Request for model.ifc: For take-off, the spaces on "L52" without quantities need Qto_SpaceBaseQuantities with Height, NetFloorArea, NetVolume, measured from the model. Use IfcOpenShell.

First a look at what the model holds.

```python
import ifcopenshell
import ifcopenshell.util.element
import ifcopenshell.util.unit

model = ifcopenshell.open("model.ifc")
print(model.schema)
for unit_type in ("LENGTHUNIT", "AREAUNIT", "VOLUMEUNIT"):
    print(unit_type, ifcopenshell.util.unit.calculate_unit_scale(model, unit_type))
storey = next(s for s in model.by_type("IfcBuildingStorey") if s.Name == "L52")
spaces = [e for e in ifcopenshell.util.element.get_decomposition(storey) if e.is_a("IfcSpace")]
for e in sorted(spaces, key=lambda e: e.id()):
    print(e.id(), e.is_a(), e.Name, list(ifcopenshell.util.element.get_psets(e, qtos_only=True)), sep=" | ")
```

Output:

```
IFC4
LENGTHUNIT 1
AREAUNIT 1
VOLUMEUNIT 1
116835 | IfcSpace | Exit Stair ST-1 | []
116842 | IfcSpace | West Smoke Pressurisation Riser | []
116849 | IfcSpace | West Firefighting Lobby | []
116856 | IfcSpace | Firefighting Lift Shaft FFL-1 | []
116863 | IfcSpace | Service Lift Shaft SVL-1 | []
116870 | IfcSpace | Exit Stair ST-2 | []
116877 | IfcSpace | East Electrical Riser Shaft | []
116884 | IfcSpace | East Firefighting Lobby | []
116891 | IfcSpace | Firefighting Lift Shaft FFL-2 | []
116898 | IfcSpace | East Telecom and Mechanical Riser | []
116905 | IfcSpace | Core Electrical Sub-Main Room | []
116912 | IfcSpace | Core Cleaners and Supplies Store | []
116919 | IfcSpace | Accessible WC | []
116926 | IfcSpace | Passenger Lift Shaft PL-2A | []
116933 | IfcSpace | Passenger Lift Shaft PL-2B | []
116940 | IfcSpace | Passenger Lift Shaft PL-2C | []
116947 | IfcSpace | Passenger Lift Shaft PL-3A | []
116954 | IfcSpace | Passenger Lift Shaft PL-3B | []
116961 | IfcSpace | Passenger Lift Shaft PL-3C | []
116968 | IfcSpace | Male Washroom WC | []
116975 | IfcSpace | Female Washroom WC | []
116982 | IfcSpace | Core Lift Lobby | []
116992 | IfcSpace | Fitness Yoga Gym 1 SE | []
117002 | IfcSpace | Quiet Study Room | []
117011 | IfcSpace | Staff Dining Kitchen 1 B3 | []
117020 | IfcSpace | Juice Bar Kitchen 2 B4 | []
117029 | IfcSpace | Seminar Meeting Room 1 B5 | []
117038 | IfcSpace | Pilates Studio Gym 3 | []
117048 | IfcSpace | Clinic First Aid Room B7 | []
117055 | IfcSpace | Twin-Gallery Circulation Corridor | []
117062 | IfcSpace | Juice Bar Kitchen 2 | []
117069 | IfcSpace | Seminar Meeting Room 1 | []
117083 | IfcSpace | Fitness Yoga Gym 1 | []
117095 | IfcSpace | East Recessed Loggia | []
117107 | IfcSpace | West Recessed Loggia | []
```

```python
import ifcopenshell
import ifcopenshell.api.pset
import ifcopenshell.geom
import ifcopenshell.util.element
import ifcopenshell.util.shape
import ifcopenshell.util.unit

model = ifcopenshell.open("model.ifc")
unit_scale = ifcopenshell.util.unit.calculate_unit_scale(model)
area_scale = ifcopenshell.util.unit.calculate_unit_scale(model, "AREAUNIT")
volume_scale = ifcopenshell.util.unit.calculate_unit_scale(model, "VOLUMEUNIT")
settings = ifcopenshell.geom.settings()

storey = next(s for s in model.by_type("IfcBuildingStorey") if s.Name == "L52")
spaces = [e for e in ifcopenshell.util.element.get_decomposition(storey) if e.is_a("IfcSpace")]

for e in sorted(spaces, key=lambda e: e.id()):
    if ifcopenshell.util.element.get_psets(e, qtos_only=True, should_inherit=False):
        continue
    # Geometry comes back in metres, in the element's own axes.
    shape = ifcopenshell.geom.create_shape(settings, e)
    values = {
        "Height": ifcopenshell.util.shape.get_z(shape.geometry) / unit_scale,
        "NetFloorArea": ifcopenshell.util.shape.get_footprint_area(shape.geometry) / area_scale,
        "NetVolume": ifcopenshell.util.shape.get_volume(shape.geometry) / volume_scale,
    }
    qto = ifcopenshell.api.pset.add_qto(model, product=e, name="Qto_SpaceBaseQuantities")
    ifcopenshell.api.pset.edit_qto(model, qto=qto, properties=values)
    print(e.id(), {k: round(v, 3) for k, v in values.items()})

model.write("model_updated.ifc")
```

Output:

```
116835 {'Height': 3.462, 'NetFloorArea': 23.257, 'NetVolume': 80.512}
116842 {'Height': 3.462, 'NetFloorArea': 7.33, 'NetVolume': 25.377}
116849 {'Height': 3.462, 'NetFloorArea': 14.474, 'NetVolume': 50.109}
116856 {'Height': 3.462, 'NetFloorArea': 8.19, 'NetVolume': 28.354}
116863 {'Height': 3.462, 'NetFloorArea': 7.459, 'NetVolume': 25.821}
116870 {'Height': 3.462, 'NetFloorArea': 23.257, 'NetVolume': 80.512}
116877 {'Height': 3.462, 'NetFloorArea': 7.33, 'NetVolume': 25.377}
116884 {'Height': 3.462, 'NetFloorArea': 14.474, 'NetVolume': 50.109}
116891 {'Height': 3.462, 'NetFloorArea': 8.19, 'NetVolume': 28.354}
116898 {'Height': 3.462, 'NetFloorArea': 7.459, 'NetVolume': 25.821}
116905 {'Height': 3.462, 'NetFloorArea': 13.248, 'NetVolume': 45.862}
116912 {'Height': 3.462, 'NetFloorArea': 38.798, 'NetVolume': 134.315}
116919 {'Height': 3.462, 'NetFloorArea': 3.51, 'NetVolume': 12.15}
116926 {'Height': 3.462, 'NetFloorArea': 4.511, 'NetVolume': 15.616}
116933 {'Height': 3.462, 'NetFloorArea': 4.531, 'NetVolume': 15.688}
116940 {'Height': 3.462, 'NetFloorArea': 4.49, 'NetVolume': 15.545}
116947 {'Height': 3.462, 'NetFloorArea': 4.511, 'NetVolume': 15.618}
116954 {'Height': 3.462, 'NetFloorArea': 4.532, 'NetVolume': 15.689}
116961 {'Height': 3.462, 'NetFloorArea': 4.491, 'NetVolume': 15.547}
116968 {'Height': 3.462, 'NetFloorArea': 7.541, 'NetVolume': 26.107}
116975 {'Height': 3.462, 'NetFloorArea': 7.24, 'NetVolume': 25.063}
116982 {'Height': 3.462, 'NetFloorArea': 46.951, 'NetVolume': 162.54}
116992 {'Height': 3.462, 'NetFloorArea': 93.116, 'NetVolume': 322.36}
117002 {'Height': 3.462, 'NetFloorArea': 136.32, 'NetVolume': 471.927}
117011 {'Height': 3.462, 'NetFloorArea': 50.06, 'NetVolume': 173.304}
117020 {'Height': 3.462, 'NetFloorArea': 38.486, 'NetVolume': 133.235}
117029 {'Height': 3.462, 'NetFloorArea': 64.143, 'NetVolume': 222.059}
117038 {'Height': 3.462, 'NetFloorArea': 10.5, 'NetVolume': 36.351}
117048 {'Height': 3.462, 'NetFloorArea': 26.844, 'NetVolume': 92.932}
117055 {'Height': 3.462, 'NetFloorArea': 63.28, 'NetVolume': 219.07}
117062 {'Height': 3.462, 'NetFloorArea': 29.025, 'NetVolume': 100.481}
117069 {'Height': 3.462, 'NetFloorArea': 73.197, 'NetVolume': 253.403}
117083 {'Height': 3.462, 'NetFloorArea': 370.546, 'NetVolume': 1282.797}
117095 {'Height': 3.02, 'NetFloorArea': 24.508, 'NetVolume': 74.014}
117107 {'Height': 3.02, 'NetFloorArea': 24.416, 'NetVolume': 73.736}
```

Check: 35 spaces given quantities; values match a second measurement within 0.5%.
